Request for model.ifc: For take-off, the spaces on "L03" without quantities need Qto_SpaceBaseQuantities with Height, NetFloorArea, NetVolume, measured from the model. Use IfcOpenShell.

First a look at what the model holds.

```python
import ifcopenshell
import ifcopenshell.util.element
import ifcopenshell.util.unit

model = ifcopenshell.open("model.ifc")
print(model.schema)
for unit_type in ("LENGTHUNIT", "AREAUNIT", "VOLUMEUNIT"):
    print(unit_type, ifcopenshell.util.unit.calculate_unit_scale(model, unit_type))
storey = next(s for s in model.by_type("IfcBuildingStorey") if s.Name == "L03")
spaces = [e for e in ifcopenshell.util.element.get_decomposition(storey) if e.is_a("IfcSpace")]
for e in sorted(spaces, key=lambda e: e.id()):
    print(e.id(), e.is_a(), e.Name, list(ifcopenshell.util.element.get_psets(e, qtos_only=True)), sep=" | ")
```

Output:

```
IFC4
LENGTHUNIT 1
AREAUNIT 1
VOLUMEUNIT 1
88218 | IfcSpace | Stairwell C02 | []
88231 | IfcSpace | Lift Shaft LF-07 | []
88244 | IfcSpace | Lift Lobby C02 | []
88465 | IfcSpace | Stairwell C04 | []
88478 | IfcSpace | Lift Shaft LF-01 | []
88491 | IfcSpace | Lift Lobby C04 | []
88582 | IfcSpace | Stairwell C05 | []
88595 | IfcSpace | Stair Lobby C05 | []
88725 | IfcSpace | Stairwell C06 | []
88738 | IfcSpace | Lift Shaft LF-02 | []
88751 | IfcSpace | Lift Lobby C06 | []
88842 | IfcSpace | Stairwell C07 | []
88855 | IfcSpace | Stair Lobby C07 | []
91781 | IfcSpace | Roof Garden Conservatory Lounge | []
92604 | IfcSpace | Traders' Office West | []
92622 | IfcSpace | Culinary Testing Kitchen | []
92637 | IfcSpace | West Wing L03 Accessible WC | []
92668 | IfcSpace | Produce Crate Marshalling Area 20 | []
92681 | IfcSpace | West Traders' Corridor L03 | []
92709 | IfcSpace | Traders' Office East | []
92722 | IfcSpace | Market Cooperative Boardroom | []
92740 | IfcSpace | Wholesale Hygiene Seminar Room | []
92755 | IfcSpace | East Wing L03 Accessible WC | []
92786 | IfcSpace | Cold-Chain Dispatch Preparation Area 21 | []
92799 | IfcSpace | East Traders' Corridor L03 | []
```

```python
import ifcopenshell
import ifcopenshell.api.pset
import ifcopenshell.geom
import ifcopenshell.util.element
import ifcopenshell.util.shape
import ifcopenshell.util.unit

model = ifcopenshell.open("model.ifc")
unit_scale = ifcopenshell.util.unit.calculate_unit_scale(model)
area_scale = ifcopenshell.util.unit.calculate_unit_scale(model, "AREAUNIT")
volume_scale = ifcopenshell.util.unit.calculate_unit_scale(model, "VOLUMEUNIT")
settings = ifcopenshell.geom.settings()

storey = next(s for s in model.by_type("IfcBuildingStorey") if s.Name == "L03")
spaces = [e for e in ifcopenshell.util.element.get_decomposition(storey) if e.is_a("IfcSpace")]

for e in sorted(spaces, key=lambda e: e.id()):
    if ifcopenshell.util.element.get_psets(e, qtos_only=True, should_inherit=False):
        continue
    # Geometry comes back in metres, in the element's own axes.
    shape = ifcopenshell.geom.create_shape(settings, e)
    values = {
        "Height": ifcopenshell.util.shape.get_z(shape.geometry) / unit_scale,
        "NetFloorArea": ifcopenshell.util.shape.get_footprint_area(shape.geometry) / area_scale,
        "NetVolume": ifcopenshell.util.shape.get_volume(shape.geometry) / volume_scale,
    }
    qto = ifcopenshell.api.pset.add_qto(model, product=e, name="Qto_SpaceBaseQuantities")
    ifcopenshell.api.pset.edit_qto(model, qto=qto, properties=values)
    print(e.id(), {k: round(v, 3) for k, v in values.items()})

model.write("model-out.ifc")
```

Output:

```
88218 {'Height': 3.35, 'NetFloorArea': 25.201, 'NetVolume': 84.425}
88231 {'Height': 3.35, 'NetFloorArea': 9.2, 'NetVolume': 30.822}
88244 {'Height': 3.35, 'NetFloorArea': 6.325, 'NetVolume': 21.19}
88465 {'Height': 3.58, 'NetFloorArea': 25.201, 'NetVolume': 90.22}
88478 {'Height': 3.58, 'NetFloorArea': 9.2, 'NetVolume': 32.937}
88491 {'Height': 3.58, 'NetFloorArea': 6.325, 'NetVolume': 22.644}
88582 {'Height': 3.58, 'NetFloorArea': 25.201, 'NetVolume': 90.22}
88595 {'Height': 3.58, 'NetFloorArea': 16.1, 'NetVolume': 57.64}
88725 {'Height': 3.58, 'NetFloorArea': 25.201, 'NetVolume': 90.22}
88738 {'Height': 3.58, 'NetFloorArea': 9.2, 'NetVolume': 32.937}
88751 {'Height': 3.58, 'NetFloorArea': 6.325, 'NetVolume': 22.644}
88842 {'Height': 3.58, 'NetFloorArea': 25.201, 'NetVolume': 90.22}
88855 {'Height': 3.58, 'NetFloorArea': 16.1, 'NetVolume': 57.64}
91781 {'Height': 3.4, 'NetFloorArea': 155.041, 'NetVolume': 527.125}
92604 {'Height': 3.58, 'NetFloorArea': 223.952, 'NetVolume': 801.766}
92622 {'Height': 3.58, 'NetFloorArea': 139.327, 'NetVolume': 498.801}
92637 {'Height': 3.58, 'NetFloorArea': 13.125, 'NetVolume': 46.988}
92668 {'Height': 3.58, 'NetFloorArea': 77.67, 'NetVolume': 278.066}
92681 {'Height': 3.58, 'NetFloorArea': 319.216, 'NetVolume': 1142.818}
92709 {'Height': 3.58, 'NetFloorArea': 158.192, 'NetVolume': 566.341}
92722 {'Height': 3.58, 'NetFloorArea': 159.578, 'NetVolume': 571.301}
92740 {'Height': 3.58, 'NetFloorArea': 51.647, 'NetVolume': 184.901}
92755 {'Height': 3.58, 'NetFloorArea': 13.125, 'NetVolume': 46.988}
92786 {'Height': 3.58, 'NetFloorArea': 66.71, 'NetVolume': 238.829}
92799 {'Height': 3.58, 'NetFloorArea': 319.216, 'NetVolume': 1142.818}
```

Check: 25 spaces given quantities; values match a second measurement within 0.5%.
